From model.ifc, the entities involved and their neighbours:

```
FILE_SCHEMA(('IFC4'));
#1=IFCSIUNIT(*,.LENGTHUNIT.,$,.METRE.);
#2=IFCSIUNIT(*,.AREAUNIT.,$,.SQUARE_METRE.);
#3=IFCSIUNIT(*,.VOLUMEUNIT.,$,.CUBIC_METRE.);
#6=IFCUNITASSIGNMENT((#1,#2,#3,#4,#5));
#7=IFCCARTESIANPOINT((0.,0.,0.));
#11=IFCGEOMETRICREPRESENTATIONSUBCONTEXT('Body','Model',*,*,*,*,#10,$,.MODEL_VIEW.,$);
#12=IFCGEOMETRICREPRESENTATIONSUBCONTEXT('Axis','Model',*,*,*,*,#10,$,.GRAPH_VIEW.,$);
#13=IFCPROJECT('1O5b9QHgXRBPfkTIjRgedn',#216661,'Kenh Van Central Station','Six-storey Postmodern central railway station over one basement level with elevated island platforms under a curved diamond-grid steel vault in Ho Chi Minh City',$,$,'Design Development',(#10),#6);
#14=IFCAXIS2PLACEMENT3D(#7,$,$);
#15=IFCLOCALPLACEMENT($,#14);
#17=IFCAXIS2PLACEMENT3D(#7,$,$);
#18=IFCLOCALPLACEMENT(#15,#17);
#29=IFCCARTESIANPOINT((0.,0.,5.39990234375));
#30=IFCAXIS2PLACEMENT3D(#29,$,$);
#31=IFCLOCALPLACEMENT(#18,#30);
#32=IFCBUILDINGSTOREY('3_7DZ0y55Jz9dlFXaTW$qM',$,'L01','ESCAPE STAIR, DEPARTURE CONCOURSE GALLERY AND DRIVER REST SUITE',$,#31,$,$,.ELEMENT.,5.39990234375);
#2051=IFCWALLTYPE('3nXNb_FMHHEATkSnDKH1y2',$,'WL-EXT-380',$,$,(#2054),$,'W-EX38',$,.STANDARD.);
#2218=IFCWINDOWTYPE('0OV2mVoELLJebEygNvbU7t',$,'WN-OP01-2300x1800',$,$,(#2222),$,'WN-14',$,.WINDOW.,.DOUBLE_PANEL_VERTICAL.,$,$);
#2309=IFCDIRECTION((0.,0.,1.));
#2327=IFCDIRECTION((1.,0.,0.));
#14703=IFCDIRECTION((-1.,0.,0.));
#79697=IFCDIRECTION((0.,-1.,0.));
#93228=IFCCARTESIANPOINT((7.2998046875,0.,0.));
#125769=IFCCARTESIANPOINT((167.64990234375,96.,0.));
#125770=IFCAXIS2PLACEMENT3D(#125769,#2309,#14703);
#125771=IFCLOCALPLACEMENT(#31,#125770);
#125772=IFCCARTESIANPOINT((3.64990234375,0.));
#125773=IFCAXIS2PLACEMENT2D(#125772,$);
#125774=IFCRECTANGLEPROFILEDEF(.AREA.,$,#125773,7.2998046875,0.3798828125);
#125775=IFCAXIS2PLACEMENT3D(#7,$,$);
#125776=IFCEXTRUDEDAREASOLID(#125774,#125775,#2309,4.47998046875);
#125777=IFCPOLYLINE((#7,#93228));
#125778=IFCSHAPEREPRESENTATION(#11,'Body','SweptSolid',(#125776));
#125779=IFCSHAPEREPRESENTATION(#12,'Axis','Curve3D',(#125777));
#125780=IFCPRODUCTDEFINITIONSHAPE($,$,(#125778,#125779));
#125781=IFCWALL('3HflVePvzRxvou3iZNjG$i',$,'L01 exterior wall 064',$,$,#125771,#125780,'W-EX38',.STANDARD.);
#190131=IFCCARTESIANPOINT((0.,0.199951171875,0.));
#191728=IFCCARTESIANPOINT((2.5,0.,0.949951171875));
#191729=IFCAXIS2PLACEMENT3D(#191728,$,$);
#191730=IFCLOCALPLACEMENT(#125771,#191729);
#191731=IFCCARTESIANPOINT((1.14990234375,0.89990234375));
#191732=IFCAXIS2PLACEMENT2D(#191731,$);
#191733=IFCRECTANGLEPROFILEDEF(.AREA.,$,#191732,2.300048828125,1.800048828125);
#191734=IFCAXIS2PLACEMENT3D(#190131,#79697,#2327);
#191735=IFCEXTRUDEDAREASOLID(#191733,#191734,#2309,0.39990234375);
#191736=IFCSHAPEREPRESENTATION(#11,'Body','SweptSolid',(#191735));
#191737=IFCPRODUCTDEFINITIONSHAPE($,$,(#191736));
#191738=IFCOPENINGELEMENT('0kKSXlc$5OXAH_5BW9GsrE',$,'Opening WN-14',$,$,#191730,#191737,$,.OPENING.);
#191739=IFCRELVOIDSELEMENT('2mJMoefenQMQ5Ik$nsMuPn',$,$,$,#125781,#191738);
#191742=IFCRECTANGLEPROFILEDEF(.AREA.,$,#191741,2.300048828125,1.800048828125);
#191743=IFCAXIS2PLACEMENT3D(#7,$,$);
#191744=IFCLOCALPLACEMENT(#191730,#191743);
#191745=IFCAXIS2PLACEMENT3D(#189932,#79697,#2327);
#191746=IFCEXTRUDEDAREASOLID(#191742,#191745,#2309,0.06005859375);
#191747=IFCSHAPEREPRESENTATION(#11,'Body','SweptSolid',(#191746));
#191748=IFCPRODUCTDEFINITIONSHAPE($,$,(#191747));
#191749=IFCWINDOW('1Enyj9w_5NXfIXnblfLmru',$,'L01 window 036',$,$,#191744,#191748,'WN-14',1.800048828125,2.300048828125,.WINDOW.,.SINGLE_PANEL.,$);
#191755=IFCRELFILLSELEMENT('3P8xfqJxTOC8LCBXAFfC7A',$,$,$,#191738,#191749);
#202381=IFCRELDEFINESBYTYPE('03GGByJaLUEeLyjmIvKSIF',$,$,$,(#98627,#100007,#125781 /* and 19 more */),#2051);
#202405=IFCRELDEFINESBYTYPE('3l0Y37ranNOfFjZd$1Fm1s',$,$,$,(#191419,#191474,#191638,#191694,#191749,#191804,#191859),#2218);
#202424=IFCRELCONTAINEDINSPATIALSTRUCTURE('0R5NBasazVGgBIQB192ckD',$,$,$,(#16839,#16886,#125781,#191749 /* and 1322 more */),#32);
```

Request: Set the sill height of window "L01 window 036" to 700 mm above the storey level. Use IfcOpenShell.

```python
import numpy as np
import ifcopenshell
import ifcopenshell.api.geometry
import ifcopenshell.geom
import ifcopenshell.util.element
import ifcopenshell.util.placement
import ifcopenshell.util.shape
import ifcopenshell.util.unit

model = ifcopenshell.open("model.ifc")
unit_scale = ifcopenshell.util.unit.calculate_unit_scale(model)

window = model.by_guid("1Enyj9w_5NXfIXnblfLmru")
opening = window.FillsVoids[0].RelatingOpeningElement
storey = ifcopenshell.util.element.get_container(window, ifc_class="IfcBuildingStorey")
level = ifcopenshell.util.placement.get_local_placement(storey.ObjectPlacement)[2, 3]

# The opening's origin need not be at the sill, so measure its lowest point.
shape = ifcopenshell.geom.create_shape(ifcopenshell.geom.settings(), opening)
bottom = ifcopenshell.util.shape.get_shape_bottom_elevation(shape, shape.geometry) / unit_scale
dz = level + 0.7 / unit_scale - bottom

shift = np.array([0.0, 0.0, dz])
# The window is placed relative to its opening, so it follows when the opening moves.
matrix = ifcopenshell.util.placement.get_local_placement(opening.ObjectPlacement)
matrix[:3, 3] += shift
ifcopenshell.api.geometry.edit_object_placement(
    model, product=opening, matrix=matrix, is_si=False, should_transform_children=True
)

print(f"moved by {dz * unit_scale:+.3f} m")

model.write("model_v2.ifc")
```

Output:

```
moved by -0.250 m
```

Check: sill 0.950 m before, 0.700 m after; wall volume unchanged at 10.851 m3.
